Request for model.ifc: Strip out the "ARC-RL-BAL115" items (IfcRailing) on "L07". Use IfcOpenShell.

First a look at what the model holds.

```python
import ifcopenshell
import ifcopenshell.util.element

model = ifcopenshell.open("model.ifc")
print(model.schema)
storey = next(s for s in model.by_type("IfcBuildingStorey") if s.Name == "L07")
railings = [e for e in ifcopenshell.util.element.get_decomposition(storey) if e.is_a("IfcRailing")]
seen = {}
for e in railings:
    element_type = ifcopenshell.util.element.get_type(e)
    name = element_type.Name if element_type not in (None, e) else None
    seen[name] = seen.get(name, 0) + 1
for name, count in sorted(seen.items(), key=str):
    print(count, "x", name)
```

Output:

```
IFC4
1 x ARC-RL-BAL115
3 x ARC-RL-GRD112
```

```python
import ifcopenshell
import ifcopenshell.api.root
import ifcopenshell.util.element

model = ifcopenshell.open("model.ifc")

storey = next(s for s in model.by_type("IfcBuildingStorey") if s.Name == "L07")
railings = [e for e in ifcopenshell.util.element.get_decomposition(storey) if e.is_a("IfcRailing")]
targets = [e for e in railings if (t := ifcopenshell.util.element.get_type(e)) not in (None, e) and t.Name == "ARC-RL-BAL115"]

for e in targets:
    ifcopenshell.api.root.remove_product(model, product=e)
print(len(targets), "removed")

model.write("model_v2.ifc")
```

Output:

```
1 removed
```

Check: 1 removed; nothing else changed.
